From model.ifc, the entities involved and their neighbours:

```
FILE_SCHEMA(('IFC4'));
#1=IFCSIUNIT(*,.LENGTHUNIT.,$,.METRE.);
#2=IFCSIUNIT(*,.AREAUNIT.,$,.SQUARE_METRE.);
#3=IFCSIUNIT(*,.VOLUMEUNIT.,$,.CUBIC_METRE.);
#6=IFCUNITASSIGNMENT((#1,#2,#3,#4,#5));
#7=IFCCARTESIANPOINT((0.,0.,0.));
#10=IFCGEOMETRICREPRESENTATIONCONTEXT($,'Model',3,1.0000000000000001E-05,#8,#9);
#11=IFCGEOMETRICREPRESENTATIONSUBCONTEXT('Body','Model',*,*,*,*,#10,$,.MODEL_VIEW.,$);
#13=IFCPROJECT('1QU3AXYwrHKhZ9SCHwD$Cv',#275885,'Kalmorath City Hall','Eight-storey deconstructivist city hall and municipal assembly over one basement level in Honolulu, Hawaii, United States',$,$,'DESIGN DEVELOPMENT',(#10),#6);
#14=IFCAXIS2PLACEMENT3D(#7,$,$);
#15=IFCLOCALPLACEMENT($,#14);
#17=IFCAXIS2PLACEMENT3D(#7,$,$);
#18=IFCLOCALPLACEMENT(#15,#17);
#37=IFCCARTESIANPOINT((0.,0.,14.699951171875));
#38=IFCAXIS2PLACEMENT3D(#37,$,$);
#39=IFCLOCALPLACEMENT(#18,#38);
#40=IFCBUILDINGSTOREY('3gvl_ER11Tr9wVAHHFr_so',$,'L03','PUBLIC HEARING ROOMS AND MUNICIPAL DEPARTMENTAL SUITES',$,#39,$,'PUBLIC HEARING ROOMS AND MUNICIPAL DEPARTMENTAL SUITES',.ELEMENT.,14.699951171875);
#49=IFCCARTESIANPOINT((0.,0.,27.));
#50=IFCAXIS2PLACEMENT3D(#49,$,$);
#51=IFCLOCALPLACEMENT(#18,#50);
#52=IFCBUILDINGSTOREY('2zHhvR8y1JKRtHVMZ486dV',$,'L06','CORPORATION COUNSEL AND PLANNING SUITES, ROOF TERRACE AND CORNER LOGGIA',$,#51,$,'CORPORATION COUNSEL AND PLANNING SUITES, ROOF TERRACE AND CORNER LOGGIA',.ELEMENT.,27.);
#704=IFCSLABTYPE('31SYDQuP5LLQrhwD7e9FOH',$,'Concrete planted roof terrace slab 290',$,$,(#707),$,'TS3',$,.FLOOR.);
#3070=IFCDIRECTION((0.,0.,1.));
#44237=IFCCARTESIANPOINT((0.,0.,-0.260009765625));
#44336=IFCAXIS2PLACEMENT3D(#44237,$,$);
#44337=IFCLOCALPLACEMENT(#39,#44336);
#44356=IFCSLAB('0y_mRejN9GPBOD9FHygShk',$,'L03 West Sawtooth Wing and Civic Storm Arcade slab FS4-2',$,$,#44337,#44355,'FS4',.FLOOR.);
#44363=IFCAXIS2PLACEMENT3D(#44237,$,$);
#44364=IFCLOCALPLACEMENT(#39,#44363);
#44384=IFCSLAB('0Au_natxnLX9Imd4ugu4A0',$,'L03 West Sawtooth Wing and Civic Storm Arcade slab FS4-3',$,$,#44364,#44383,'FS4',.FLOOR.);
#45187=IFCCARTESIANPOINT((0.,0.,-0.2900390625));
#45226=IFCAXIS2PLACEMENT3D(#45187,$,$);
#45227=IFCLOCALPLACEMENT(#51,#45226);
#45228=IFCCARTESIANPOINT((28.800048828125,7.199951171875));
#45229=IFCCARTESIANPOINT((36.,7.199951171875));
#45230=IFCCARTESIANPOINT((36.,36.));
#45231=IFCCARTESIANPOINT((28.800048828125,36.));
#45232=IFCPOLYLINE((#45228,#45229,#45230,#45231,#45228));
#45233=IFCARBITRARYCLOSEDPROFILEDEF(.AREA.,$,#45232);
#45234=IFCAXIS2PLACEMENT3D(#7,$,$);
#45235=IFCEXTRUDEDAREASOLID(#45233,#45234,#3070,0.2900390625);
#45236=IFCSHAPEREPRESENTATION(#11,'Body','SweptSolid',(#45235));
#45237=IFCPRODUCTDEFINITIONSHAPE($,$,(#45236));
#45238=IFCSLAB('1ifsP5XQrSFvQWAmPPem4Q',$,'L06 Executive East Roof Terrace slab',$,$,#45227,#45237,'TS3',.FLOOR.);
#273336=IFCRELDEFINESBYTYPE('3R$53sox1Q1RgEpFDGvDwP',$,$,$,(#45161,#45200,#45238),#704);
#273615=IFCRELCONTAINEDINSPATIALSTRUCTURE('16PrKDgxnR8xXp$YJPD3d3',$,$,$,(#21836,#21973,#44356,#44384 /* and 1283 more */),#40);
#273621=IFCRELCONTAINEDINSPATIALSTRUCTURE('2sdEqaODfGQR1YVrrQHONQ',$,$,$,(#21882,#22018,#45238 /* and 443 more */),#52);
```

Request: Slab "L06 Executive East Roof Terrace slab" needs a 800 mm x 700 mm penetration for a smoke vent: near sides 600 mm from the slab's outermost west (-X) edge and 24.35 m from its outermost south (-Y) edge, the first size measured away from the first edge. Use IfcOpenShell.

```python
import numpy as np
import ifcopenshell
import ifcopenshell.api.feature
import ifcopenshell.api.geometry
import ifcopenshell.api.root
import ifcopenshell.geom
import ifcopenshell.util.placement
import ifcopenshell.util.representation
import ifcopenshell.util.shape
import ifcopenshell.util.unit

model = ifcopenshell.open("model.ifc")
unit_scale = ifcopenshell.util.unit.calculate_unit_scale(model)
settings = ifcopenshell.geom.settings()


def volume(element):
    """Net volume in cubic metres, openings subtracted."""
    shape = ifcopenshell.geom.create_shape(settings, element)
    return ifcopenshell.util.shape.get_volume(shape.geometry)


slab = model.by_guid("1ifsP5XQrSFvQWAmPPem4Q")
before = volume(slab)

# Extent in the slab's own axes, in metres. The edges named are its -X and -Y sides.
slab_shape = ifcopenshell.geom.create_shape(settings, slab)
vertices = ifcopenshell.util.shape.get_vertices(slab_shape.geometry)
x_min, y_min, bottom = vertices.min(axis=0)
top = vertices[:, 2].max()

opening = ifcopenshell.api.root.create_entity(model, ifc_class="IfcOpeningElement", name="Smoke vent opening", predefined_type="OPENING")
context = ifcopenshell.util.representation.get_context(model, "Model", "Body", "MODEL_VIEW")
width, depth = 0.8, 0.7
outline = [(0.0, 0.0), (width, 0.0), (width, depth), (0.0, depth), (0.0, 0.0)]
# Overshoot both faces by 50 mm so the cut is clean.
shape = ifcopenshell.api.geometry.add_slab_representation(
    model, context=context, depth=top - bottom + 0.1, polyline=outline
)
ifcopenshell.api.geometry.assign_representation(model, product=opening, representation=shape)

matrix = ifcopenshell.util.placement.get_local_placement(slab.ObjectPlacement)
matrix[:, 3] = matrix @ np.append(np.array([x_min + 0.6, y_min + 24.35, bottom - 0.05]) / unit_scale, 1.0)
ifcopenshell.api.geometry.edit_object_placement(model, product=opening, matrix=matrix, is_si=False)
ifcopenshell.api.feature.add_feature(model, feature=opening, element=slab)

after = volume(slab)

print(f"slab volume {before:.3f} -> {after:.3f} m3")

model.write("model_updated.ifc")
```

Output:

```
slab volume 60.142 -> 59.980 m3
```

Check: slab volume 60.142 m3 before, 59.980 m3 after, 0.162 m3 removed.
